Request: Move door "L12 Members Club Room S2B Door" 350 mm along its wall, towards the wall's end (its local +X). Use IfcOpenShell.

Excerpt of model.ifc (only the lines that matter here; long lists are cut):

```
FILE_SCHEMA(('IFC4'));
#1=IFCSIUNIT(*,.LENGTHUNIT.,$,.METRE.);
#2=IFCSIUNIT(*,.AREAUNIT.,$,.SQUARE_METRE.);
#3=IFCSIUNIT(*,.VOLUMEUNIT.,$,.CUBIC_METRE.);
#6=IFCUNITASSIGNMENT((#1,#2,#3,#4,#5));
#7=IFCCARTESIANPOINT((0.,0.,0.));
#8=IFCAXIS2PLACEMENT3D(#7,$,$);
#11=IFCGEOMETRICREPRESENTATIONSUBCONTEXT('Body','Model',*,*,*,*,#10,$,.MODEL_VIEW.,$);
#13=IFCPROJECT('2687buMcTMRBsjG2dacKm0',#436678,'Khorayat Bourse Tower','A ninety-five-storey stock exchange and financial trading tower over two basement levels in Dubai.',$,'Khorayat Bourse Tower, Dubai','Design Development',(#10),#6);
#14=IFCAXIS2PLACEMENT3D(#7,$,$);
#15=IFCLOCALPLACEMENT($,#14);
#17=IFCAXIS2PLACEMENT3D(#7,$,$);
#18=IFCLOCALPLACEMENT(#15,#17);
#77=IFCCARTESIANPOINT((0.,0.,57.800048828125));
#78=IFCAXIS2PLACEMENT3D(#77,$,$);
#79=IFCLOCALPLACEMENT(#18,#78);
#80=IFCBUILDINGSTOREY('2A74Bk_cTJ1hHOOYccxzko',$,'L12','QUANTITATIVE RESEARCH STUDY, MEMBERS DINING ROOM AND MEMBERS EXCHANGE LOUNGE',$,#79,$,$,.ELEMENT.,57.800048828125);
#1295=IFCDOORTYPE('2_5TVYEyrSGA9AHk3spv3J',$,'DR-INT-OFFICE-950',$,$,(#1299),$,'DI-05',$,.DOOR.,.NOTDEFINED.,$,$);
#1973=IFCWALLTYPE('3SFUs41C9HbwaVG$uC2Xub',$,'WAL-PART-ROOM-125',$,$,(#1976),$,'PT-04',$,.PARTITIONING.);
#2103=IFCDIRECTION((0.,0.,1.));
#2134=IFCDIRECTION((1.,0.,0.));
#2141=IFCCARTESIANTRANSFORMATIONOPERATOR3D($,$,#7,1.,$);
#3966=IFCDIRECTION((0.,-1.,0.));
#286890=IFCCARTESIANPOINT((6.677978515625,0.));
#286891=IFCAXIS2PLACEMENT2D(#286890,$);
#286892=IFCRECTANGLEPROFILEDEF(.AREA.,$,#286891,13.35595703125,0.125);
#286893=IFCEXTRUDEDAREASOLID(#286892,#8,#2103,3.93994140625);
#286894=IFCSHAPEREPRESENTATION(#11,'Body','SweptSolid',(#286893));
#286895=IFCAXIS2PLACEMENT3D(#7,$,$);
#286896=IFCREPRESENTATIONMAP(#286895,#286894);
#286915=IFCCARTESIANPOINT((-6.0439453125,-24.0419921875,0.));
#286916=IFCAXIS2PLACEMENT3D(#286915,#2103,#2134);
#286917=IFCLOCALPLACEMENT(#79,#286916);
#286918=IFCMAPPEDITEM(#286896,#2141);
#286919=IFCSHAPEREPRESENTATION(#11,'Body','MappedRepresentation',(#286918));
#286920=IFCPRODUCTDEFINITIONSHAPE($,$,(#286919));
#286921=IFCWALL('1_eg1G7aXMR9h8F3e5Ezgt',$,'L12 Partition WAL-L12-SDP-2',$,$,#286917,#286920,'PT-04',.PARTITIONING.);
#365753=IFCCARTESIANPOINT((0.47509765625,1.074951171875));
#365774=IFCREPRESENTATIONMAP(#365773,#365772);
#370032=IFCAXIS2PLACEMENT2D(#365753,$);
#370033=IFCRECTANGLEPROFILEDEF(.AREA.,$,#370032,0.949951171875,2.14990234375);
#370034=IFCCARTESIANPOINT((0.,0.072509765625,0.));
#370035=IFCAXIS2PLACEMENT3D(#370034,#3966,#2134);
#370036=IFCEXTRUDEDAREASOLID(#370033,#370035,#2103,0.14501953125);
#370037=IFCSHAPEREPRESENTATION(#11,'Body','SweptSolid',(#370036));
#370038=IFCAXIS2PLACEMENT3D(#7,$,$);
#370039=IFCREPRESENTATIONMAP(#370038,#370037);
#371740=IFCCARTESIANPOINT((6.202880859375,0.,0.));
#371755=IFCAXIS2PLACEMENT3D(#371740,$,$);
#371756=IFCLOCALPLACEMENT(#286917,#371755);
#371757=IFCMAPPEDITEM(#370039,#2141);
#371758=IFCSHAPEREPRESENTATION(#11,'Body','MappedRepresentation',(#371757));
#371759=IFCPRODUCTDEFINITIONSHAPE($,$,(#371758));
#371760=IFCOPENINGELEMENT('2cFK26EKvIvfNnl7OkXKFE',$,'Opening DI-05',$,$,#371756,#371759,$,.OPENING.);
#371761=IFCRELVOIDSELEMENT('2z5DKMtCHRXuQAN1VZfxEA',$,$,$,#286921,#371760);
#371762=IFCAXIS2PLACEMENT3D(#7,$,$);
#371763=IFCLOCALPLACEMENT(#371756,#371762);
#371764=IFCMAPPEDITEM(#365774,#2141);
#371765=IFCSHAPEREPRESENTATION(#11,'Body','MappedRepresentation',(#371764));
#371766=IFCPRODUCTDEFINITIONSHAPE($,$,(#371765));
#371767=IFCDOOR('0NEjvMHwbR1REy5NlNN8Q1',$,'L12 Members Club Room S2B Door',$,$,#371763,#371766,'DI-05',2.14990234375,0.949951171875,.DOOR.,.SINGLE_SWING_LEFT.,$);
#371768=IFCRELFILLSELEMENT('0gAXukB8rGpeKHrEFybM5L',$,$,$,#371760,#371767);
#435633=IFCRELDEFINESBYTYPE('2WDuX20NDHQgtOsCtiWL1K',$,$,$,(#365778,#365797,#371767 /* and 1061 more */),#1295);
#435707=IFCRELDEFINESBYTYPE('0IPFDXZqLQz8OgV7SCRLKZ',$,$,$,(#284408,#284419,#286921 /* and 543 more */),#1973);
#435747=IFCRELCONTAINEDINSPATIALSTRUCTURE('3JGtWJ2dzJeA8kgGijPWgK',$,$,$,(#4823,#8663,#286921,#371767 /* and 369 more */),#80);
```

```python
import ifcopenshell
import ifcopenshell.api.geometry
import ifcopenshell.util.placement
import ifcopenshell.util.unit

model = ifcopenshell.open("model.ifc")
unit_scale = ifcopenshell.util.unit.calculate_unit_scale(model)

door = model.by_guid("0NEjvMHwbR1REy5NlNN8Q1")
opening = door.FillsVoids[0].RelatingOpeningElement
wall = opening.VoidsElements[0].RelatingBuildingElement

wall_matrix = ifcopenshell.util.placement.get_local_placement(wall.ObjectPlacement)
shift = wall_matrix[:3, 0] * 0.35 / unit_scale
before = ifcopenshell.util.placement.get_local_placement(door.ObjectPlacement)[:3, 3].copy()

# The door is placed relative to its opening, so it follows when the opening moves.
matrix = ifcopenshell.util.placement.get_local_placement(opening.ObjectPlacement)
matrix[:3, 3] += shift
ifcopenshell.api.geometry.edit_object_placement(
    model, product=opening, matrix=matrix, is_si=False, should_transform_children=True
)

after = ifcopenshell.util.placement.get_local_placement(door.ObjectPlacement)[:3, 3]
print("door moved by", (after - before).round(3) + 0.0)

model.write("model_edited.ifc")
```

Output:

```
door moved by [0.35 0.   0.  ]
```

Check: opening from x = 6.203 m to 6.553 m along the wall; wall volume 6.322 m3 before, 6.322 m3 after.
